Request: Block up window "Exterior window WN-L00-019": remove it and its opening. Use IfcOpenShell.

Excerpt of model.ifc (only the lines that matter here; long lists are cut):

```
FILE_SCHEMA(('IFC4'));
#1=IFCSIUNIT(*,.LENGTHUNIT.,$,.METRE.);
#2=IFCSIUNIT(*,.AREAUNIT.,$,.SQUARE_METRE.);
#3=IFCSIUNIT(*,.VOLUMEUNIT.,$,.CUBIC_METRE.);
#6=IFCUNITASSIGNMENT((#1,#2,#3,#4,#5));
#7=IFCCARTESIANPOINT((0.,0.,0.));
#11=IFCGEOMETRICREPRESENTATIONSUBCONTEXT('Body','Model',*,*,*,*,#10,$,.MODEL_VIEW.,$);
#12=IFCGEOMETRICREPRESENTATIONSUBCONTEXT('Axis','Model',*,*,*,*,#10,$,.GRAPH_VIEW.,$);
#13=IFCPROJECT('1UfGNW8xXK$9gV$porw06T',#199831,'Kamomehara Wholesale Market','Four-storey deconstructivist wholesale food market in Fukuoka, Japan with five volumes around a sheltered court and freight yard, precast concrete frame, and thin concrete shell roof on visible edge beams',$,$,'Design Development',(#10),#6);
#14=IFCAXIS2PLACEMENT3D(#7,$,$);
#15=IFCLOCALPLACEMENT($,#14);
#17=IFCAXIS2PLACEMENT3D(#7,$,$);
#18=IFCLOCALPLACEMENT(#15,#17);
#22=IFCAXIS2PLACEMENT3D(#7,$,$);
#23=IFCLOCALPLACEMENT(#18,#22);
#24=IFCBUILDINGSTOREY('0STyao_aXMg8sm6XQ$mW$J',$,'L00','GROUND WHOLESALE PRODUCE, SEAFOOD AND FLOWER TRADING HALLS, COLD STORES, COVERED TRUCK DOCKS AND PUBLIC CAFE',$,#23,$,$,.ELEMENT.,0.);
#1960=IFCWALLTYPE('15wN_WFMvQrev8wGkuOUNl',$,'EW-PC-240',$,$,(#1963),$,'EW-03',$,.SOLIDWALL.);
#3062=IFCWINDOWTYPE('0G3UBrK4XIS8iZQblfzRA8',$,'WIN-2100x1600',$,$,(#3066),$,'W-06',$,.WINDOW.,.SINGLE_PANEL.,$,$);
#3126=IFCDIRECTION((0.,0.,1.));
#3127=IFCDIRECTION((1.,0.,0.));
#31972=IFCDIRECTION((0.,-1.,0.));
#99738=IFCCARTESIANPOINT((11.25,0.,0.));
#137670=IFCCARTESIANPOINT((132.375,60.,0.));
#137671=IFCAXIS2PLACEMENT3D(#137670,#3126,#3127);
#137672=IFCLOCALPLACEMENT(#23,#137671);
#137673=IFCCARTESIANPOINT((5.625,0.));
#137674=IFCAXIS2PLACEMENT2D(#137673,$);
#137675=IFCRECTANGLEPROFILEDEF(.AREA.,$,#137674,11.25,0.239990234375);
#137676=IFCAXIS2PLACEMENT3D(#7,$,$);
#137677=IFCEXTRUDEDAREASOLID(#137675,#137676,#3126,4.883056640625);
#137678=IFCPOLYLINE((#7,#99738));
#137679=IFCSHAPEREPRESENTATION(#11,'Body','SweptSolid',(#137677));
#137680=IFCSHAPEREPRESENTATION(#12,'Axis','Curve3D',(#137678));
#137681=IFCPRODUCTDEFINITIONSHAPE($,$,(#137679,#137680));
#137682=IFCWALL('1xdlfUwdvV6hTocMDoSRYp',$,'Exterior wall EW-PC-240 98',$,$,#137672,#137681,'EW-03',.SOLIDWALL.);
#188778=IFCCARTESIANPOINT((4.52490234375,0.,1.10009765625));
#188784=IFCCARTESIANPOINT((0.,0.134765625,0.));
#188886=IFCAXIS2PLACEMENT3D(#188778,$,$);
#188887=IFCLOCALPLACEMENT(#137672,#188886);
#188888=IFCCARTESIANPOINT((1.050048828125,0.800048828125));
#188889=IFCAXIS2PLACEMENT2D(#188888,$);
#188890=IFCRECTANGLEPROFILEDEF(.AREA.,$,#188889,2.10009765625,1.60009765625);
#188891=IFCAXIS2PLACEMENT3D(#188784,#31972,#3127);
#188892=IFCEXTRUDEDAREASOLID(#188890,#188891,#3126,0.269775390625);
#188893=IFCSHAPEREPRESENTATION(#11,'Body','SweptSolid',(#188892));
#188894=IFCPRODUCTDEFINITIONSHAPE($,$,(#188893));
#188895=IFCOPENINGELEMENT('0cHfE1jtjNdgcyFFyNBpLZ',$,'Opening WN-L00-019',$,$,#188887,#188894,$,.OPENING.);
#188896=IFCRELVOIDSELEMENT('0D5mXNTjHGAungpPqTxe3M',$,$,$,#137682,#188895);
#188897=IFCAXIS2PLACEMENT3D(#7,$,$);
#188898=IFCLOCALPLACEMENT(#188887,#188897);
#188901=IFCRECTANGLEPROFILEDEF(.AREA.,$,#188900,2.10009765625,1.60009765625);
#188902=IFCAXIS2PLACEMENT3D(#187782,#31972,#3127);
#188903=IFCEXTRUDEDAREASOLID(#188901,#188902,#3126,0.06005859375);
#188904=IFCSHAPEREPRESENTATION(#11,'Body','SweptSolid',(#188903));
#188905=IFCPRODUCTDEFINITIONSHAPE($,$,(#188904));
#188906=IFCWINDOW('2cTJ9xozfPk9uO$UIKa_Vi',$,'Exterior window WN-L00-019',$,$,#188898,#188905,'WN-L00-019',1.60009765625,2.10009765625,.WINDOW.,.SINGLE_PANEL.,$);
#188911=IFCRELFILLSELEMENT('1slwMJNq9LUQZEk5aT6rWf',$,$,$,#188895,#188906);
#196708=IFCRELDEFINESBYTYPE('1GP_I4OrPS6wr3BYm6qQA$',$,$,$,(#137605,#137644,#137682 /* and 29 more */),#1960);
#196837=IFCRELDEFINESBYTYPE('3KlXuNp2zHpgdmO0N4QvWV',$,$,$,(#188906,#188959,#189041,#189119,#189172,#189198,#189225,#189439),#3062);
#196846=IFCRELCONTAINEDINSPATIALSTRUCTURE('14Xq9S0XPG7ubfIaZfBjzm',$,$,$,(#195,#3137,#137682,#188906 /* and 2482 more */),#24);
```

```python
import ifcopenshell
import ifcopenshell.api.feature
import ifcopenshell.api.root
import ifcopenshell.geom
import ifcopenshell.util.shape

model = ifcopenshell.open("model.ifc")
settings = ifcopenshell.geom.settings()


def volume(element):
    """Net volume in cubic metres, openings subtracted."""
    shape = ifcopenshell.geom.create_shape(settings, element)
    return ifcopenshell.util.shape.get_volume(shape.geometry)


window = model.by_id(188906)
opening = window.FillsVoids[0].RelatingOpeningElement
wall = opening.VoidsElements[0].RelatingBuildingElement
before = volume(wall)

ifcopenshell.api.root.remove_product(model, product=window)
ifcopenshell.api.feature.remove_feature(model, feature=opening)

after = volume(wall)

print(f"wall volume {before:.3f} -> {after:.3f} m3")

model.write("model-out.ifc")
```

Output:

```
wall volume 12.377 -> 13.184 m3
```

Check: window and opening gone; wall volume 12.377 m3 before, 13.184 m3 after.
